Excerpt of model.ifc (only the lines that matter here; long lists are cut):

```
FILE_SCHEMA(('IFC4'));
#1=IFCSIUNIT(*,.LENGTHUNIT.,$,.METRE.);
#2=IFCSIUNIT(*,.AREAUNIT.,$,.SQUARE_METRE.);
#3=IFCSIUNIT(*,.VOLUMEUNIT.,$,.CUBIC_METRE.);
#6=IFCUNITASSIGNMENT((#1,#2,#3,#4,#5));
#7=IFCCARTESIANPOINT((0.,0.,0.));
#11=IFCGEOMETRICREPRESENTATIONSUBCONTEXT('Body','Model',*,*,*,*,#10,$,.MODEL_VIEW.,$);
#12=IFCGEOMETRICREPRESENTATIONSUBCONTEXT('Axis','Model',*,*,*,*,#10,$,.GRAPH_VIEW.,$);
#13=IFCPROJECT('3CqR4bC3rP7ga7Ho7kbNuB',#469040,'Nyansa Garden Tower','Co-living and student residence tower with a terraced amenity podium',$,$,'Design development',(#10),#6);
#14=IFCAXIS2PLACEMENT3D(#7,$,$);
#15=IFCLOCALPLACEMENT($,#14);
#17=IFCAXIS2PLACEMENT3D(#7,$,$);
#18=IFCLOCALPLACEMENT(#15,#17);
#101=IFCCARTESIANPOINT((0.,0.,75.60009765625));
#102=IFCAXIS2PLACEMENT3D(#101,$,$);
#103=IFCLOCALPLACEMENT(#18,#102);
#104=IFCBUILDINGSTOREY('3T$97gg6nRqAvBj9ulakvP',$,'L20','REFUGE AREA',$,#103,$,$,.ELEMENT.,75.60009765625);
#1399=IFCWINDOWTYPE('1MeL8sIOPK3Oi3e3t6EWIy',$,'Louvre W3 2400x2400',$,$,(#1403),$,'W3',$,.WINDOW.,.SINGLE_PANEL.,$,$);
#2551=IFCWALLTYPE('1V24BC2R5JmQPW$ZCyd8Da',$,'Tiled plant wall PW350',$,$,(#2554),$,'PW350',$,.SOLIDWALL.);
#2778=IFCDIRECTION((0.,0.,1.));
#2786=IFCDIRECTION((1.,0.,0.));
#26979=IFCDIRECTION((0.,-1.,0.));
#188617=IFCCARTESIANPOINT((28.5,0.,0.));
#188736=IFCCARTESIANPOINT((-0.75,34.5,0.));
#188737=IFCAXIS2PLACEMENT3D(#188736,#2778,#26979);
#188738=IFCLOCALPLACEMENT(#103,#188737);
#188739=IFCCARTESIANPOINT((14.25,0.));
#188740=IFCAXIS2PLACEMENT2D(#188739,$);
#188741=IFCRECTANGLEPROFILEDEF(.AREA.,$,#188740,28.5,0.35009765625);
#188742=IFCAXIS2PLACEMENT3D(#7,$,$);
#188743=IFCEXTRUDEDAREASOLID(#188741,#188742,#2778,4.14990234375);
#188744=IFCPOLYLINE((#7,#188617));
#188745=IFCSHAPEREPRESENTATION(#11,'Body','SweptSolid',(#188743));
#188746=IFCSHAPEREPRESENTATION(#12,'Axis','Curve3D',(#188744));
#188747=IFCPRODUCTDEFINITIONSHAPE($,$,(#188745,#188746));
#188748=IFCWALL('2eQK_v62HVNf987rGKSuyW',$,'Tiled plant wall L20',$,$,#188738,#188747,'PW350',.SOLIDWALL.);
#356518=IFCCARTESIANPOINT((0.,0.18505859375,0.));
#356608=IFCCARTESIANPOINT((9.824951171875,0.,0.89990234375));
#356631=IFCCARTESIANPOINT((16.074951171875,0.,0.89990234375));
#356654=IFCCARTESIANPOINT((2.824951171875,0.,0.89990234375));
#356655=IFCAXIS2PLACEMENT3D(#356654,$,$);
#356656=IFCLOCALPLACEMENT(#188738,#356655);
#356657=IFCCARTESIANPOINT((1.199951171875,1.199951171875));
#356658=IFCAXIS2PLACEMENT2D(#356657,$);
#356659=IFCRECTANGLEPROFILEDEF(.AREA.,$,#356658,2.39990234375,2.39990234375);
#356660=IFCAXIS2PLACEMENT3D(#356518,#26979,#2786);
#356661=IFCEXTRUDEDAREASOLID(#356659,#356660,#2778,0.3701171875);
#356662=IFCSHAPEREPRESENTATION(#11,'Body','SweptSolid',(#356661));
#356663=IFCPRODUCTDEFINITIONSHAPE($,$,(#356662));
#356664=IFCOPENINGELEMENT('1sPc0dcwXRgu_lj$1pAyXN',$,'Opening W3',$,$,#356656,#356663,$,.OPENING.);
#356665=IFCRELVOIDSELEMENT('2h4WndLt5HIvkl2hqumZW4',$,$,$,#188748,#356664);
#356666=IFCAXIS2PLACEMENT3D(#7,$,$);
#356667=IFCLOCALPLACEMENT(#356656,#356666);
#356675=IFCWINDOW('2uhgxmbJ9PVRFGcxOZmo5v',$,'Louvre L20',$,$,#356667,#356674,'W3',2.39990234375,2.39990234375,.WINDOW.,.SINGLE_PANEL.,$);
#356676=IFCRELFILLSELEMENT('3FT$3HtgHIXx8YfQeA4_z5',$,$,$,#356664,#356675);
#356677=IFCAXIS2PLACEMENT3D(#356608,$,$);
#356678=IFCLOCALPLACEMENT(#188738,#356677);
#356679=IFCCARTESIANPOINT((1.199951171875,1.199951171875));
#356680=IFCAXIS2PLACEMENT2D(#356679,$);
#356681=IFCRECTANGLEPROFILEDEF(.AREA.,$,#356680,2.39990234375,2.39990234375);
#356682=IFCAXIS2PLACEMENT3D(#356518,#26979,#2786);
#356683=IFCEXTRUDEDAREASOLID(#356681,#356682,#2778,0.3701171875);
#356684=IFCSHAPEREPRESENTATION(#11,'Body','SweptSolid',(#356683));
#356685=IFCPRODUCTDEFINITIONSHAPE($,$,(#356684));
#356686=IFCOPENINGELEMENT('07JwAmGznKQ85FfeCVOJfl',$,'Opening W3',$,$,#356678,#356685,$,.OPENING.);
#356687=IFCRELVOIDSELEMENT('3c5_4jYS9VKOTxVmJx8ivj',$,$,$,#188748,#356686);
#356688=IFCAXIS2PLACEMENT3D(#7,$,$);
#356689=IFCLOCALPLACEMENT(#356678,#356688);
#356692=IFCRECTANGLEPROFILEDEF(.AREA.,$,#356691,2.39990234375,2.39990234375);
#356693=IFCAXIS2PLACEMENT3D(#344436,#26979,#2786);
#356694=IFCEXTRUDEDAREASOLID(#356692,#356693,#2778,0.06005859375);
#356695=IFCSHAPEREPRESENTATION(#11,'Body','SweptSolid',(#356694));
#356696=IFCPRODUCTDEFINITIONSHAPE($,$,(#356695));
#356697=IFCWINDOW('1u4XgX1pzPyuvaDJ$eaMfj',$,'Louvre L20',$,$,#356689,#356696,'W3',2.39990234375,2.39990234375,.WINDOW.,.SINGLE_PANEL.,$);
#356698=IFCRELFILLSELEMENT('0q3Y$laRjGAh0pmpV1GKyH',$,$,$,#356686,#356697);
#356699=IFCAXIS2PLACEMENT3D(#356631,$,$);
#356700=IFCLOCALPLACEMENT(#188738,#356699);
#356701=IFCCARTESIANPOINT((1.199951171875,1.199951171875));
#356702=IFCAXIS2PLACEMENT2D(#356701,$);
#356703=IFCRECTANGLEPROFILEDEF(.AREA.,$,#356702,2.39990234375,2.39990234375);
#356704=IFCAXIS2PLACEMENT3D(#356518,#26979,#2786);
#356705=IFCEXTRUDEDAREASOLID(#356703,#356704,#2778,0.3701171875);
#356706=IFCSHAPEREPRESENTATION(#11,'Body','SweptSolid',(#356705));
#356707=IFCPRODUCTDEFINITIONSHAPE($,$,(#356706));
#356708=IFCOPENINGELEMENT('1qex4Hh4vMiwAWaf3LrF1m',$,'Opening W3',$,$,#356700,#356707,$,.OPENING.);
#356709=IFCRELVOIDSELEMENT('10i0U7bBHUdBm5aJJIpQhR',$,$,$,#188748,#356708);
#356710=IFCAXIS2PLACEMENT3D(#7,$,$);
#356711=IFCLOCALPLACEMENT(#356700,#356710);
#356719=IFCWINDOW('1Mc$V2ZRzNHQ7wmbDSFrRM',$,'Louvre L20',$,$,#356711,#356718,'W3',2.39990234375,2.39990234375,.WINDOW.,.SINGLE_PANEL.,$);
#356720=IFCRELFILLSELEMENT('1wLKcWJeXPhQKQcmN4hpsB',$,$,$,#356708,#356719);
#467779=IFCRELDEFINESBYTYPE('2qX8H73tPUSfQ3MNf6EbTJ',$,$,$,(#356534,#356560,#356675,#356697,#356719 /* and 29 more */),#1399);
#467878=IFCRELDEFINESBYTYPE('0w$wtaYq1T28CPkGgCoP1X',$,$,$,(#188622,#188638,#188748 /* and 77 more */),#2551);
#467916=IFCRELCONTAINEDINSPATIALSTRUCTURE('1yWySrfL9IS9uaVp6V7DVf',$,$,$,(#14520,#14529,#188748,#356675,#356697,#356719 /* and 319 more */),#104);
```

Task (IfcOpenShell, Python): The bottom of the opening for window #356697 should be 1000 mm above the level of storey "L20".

```python
import numpy as np
import ifcopenshell
import ifcopenshell.api.geometry
import ifcopenshell.geom
import ifcopenshell.util.element
import ifcopenshell.util.placement
import ifcopenshell.util.shape
import ifcopenshell.util.unit

model = ifcopenshell.open("model.ifc")
unit_scale = ifcopenshell.util.unit.calculate_unit_scale(model)

window = model.by_guid("1u4XgX1pzPyuvaDJ$eaMfj")
opening = window.FillsVoids[0].RelatingOpeningElement
storey = ifcopenshell.util.element.get_container(window, ifc_class="IfcBuildingStorey")
level = ifcopenshell.util.placement.get_local_placement(storey.ObjectPlacement)[2, 3]

# The opening's origin need not be at the sill, so measure its lowest point.
shape = ifcopenshell.geom.create_shape(ifcopenshell.geom.settings(), opening)
bottom = ifcopenshell.util.shape.get_shape_bottom_elevation(shape, shape.geometry) / unit_scale
dz = level + 1.0 - bottom

shift = np.array([0.0, 0.0, dz])
# The window is placed relative to its opening, so it follows when the opening moves.
matrix = ifcopenshell.util.placement.get_local_placement(opening.ObjectPlacement)
matrix[:3, 3] += shift
ifcopenshell.api.geometry.edit_object_placement(
    model, product=opening, matrix=matrix, is_si=False, should_transform_children=True
)

print(f"moved by {dz * unit_scale:+.3f} m")

model.write("model_edited.ifc")
```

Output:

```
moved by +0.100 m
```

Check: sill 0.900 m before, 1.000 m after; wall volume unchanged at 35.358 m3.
